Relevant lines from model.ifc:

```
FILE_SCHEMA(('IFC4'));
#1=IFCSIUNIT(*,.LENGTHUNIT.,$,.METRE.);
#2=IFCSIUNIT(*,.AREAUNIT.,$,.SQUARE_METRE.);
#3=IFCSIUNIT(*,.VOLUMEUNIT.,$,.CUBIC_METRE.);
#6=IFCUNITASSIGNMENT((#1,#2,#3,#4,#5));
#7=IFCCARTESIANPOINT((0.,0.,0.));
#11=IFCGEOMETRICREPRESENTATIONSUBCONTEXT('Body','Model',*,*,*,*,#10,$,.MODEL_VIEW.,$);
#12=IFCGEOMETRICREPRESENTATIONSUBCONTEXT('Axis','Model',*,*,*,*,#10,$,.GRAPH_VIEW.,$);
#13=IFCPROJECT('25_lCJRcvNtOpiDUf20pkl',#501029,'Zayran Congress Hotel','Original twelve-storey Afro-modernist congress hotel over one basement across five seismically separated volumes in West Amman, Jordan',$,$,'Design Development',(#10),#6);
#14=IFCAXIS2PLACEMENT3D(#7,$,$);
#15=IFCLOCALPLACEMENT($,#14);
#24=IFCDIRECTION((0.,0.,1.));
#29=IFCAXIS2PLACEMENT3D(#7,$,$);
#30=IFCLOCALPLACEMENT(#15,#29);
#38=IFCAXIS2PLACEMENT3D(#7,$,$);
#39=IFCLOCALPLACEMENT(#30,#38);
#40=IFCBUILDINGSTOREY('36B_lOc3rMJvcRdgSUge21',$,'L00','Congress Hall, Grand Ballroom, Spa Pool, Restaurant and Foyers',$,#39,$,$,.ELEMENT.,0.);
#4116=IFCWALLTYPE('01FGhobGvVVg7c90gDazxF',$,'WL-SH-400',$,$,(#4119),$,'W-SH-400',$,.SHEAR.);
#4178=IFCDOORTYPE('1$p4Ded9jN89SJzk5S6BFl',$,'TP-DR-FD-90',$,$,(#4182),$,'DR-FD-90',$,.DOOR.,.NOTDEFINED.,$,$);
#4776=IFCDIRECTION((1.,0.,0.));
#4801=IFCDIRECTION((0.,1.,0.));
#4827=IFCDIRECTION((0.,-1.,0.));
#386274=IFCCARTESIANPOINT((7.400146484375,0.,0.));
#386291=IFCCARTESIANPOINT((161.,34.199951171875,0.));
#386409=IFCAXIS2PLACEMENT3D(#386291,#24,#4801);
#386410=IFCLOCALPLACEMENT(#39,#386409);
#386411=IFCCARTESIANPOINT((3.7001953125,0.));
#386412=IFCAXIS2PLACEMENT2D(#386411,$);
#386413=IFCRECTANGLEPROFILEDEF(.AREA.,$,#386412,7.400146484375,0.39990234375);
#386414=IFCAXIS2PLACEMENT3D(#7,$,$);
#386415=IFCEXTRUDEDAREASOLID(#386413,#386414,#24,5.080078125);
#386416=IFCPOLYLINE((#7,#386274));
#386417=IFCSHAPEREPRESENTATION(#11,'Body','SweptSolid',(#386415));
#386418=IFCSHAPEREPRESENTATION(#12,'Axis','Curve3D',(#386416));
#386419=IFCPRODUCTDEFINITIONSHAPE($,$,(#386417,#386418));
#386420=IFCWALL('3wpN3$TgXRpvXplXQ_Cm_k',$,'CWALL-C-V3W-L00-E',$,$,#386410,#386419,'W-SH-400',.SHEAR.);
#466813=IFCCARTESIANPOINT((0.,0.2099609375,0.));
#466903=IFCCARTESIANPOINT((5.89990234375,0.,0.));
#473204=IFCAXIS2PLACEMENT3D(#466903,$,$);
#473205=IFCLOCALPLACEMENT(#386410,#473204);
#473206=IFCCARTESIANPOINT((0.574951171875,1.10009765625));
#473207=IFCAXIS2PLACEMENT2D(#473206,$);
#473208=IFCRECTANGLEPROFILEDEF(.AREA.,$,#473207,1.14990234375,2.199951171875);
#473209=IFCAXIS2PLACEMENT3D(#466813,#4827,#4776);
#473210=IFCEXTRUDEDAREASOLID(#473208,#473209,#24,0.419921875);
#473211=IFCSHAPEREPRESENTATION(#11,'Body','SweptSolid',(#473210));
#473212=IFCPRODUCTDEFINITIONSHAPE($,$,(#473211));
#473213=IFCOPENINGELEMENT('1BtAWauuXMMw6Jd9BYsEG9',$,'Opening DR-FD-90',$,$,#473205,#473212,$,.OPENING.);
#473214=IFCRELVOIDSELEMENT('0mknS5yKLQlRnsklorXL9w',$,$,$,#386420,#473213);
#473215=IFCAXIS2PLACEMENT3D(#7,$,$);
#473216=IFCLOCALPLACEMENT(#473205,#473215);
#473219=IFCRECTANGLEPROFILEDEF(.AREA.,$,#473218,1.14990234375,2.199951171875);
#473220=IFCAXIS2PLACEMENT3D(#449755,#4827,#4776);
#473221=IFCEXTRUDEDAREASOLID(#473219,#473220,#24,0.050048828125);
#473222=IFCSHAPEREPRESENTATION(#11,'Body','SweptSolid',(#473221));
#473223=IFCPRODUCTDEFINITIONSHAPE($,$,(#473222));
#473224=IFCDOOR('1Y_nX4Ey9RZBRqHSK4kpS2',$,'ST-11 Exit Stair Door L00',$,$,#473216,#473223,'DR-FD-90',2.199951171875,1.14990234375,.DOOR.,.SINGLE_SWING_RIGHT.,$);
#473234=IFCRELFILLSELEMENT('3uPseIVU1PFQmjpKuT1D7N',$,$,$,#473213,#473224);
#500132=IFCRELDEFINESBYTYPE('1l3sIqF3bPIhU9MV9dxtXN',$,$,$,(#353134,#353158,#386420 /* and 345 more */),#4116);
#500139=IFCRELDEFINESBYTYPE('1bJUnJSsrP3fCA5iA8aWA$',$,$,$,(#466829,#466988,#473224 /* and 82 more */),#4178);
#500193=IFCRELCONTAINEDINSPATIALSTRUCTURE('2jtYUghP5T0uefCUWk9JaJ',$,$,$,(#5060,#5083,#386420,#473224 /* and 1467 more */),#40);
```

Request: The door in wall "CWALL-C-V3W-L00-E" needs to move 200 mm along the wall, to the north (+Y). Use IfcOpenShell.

```python
import ifcopenshell
import ifcopenshell.api.geometry
import ifcopenshell.util.placement
import ifcopenshell.util.unit

model = ifcopenshell.open("model.ifc")
unit_scale = ifcopenshell.util.unit.calculate_unit_scale(model)

door = model.by_guid("1Y_nX4Ey9RZBRqHSK4kpS2")
opening = door.FillsVoids[0].RelatingOpeningElement
wall = opening.VoidsElements[0].RelatingBuildingElement

wall_matrix = ifcopenshell.util.placement.get_local_placement(wall.ObjectPlacement)
shift = wall_matrix[:3, 0] * 0.2 / unit_scale
before = ifcopenshell.util.placement.get_local_placement(door.ObjectPlacement)[:3, 3].copy()

# The door is placed relative to its opening, so it follows when the opening moves.
matrix = ifcopenshell.util.placement.get_local_placement(opening.ObjectPlacement)
matrix[:3, 3] += shift
ifcopenshell.api.geometry.edit_object_placement(
    model, product=opening, matrix=matrix, is_si=False, should_transform_children=True
)

after = ifcopenshell.util.placement.get_local_placement(door.ObjectPlacement)[:3, 3]
print("door moved by", (after - before).round(3) + 0.0)

model.write("model_edited.ifc")
```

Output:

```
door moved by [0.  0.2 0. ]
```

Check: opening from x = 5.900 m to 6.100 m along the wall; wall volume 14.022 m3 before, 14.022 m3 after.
